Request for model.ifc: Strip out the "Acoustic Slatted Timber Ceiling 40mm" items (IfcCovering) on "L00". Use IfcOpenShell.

First a look at what the model holds.

```python
import ifcopenshell
import ifcopenshell.util.element

model = ifcopenshell.open("model.ifc")
print(model.schema)
storey = next(s for s in model.by_type("IfcBuildingStorey") if s.Name == "L00")
coverings = [e for e in ifcopenshell.util.element.get_decomposition(storey) if e.is_a("IfcCovering")]
seen = {}
for e in coverings:
    element_type = ifcopenshell.util.element.get_type(e)
    name = element_type.Name if element_type not in (None, e) else None
    seen[name] = seen.get(name, 0) + 1
for name, count in sorted(seen.items(), key=str):
    print(count, "x", name)
```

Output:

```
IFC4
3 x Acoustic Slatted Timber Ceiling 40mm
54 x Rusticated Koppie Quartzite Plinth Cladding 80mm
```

```python
import ifcopenshell
import ifcopenshell.api.root
import ifcopenshell.util.element

model = ifcopenshell.open("model.ifc")

storey = next(s for s in model.by_type("IfcBuildingStorey") if s.Name == "L00")
coverings = [e for e in ifcopenshell.util.element.get_decomposition(storey) if e.is_a("IfcCovering")]
targets = [e for e in coverings if (t := ifcopenshell.util.element.get_type(e)) not in (None, e) and t.Name == "Acoustic Slatted Timber Ceiling 40mm"]

for e in targets:
    ifcopenshell.api.root.remove_product(model, product=e)
print(len(targets), "removed")

model.write("model_edited.ifc")
```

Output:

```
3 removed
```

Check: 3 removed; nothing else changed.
